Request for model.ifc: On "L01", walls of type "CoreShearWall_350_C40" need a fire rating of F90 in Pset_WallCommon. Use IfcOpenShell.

First a look at what the model holds.

```python
import ifcopenshell
import ifcopenshell.util.element

model = ifcopenshell.open("model.ifc")
print(model.schema)
storey = next(s for s in model.by_type("IfcBuildingStorey") if s.Name == "L01")
walls = [e for e in ifcopenshell.util.element.get_decomposition(storey) if e.is_a("IfcWall")]
seen = {}
for e in walls:
    element_type = ifcopenshell.util.element.get_type(e)
    key = (element_type.Name if element_type != e and element_type else None, ifcopenshell.util.element.get_pset(e, "Pset_WallCommon", "FireRating"))
    seen[key] = seen.get(key, 0) + 1
for (name, value), count in sorted(seen.items(), key=str):
    print(count, "x", name, "|", value)
```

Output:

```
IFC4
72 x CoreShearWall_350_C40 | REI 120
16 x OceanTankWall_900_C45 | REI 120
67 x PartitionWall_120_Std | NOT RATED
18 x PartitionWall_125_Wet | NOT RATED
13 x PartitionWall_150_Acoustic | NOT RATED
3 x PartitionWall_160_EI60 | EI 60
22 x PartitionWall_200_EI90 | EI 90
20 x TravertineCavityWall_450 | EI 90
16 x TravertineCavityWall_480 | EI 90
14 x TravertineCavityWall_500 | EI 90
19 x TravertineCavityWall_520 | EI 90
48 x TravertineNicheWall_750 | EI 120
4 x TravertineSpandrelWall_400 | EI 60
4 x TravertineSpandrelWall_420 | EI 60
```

```python
import ifcopenshell
import ifcopenshell.api.pset
import ifcopenshell.util.element

model = ifcopenshell.open("model.ifc")

storey = next(s for s in model.by_type("IfcBuildingStorey") if s.Name == "L01")
walls = [e for e in ifcopenshell.util.element.get_decomposition(storey) if e.is_a("IfcWall")]

count = 0
for e in walls:
    element_type = ifcopenshell.util.element.get_type(e)
    if element_type in (None, e) or element_type.Name != "CoreShearWall_350_C40":
        continue
    # add_pset returns the element's existing set when there is one.
    pset = ifcopenshell.api.pset.add_pset(model, product=e, name="Pset_WallCommon")
    ifcopenshell.api.pset.edit_pset(model, pset=pset, properties={"FireRating": "F90"})
    count += 1

print(count, "walls updated")

model.write("model-out.ifc")
```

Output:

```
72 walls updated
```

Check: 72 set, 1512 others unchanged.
